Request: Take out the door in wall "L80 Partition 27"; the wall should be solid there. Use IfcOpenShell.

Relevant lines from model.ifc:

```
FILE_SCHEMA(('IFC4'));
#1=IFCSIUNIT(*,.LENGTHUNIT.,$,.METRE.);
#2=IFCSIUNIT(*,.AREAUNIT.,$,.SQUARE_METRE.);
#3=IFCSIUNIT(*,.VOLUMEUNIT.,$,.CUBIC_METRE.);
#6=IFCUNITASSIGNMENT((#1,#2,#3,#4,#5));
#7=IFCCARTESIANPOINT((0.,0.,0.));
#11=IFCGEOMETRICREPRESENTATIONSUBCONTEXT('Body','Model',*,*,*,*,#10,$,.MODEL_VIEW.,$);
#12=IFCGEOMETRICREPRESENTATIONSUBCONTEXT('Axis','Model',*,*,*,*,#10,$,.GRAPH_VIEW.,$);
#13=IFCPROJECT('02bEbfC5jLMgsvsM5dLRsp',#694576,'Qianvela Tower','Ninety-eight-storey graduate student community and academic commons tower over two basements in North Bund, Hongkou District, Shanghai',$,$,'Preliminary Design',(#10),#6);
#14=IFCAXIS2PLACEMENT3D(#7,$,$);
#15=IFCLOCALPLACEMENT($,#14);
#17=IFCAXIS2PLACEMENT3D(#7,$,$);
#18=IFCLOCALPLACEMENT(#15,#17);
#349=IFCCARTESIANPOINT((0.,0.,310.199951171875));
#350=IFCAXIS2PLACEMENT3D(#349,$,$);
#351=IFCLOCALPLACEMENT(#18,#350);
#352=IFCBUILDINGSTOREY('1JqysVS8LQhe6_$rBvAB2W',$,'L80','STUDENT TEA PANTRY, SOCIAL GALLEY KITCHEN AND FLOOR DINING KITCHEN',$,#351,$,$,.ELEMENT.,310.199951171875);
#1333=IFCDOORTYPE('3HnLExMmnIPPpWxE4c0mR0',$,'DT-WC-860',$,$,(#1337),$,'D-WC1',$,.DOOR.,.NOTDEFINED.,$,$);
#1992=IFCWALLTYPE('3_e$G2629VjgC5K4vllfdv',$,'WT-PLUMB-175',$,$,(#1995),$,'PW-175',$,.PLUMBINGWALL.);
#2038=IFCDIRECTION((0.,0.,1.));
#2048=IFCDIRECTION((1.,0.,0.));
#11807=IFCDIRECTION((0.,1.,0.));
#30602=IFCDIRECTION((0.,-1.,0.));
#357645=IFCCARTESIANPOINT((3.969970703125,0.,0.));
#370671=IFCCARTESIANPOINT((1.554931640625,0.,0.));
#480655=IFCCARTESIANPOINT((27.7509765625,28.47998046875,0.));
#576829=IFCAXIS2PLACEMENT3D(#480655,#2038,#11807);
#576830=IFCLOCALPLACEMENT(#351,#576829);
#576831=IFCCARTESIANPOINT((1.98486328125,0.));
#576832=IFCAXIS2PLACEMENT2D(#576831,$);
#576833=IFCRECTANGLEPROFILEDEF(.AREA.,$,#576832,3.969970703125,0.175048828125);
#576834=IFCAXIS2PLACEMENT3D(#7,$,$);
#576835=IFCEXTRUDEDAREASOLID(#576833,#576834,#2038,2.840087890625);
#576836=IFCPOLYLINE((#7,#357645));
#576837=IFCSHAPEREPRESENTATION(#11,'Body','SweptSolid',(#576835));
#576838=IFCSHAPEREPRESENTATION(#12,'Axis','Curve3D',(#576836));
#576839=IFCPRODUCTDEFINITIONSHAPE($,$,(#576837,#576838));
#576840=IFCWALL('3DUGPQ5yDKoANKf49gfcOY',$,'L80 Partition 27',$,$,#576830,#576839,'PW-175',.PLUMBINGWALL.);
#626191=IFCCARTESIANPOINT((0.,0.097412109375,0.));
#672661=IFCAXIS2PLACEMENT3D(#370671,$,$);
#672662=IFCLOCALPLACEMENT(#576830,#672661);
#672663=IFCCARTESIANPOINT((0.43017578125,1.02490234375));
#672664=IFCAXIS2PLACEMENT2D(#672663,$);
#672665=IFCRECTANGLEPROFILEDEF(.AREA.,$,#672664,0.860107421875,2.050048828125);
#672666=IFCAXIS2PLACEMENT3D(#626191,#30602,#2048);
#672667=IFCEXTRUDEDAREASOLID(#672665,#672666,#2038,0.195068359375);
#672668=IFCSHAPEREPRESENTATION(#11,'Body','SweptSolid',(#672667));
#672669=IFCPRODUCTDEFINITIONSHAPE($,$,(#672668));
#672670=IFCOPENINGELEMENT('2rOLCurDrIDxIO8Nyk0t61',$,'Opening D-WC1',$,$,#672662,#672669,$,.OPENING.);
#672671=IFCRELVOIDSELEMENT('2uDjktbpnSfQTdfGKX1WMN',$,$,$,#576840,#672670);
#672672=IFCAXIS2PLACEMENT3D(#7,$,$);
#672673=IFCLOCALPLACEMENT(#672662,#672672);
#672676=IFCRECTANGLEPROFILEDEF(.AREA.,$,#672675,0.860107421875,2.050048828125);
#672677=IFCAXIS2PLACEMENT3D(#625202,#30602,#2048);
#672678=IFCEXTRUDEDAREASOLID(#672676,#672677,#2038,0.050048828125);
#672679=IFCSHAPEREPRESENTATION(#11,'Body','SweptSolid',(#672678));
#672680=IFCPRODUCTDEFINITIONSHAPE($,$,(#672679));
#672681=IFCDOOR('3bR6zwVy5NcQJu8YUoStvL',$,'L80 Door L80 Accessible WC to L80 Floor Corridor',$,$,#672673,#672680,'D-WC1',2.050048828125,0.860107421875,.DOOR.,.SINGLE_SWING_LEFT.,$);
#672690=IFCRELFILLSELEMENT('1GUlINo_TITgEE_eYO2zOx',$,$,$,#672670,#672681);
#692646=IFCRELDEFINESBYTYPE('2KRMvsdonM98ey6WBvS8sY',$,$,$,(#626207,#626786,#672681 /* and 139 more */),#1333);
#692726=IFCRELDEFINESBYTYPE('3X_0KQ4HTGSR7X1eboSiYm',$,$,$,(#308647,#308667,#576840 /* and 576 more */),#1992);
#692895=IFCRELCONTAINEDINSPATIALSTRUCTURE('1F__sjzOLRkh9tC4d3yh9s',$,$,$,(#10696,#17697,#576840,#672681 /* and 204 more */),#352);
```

```python
import ifcopenshell
import ifcopenshell.api.feature
import ifcopenshell.api.root
import ifcopenshell.geom
import ifcopenshell.util.shape

model = ifcopenshell.open("model.ifc")
settings = ifcopenshell.geom.settings()


def volume(element):
    """Net volume in cubic metres, openings subtracted."""
    shape = ifcopenshell.geom.create_shape(settings, element)
    return ifcopenshell.util.shape.get_volume(shape.geometry)


door = model.by_guid("3bR6zwVy5NcQJu8YUoStvL")
opening = door.FillsVoids[0].RelatingOpeningElement
wall = opening.VoidsElements[0].RelatingBuildingElement
before = volume(wall)

ifcopenshell.api.root.remove_product(model, product=door)
ifcopenshell.api.feature.remove_feature(model, feature=opening)

after = volume(wall)

print(f"wall volume {before:.3f} -> {after:.3f} m3")

model.write("model_updated.ifc")
```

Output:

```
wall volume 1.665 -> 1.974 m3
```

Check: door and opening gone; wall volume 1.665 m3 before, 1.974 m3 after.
